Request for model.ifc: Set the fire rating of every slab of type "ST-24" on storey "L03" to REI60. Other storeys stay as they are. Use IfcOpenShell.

First a look at what the model holds.

```python
import ifcopenshell
import ifcopenshell.util.element

model = ifcopenshell.open("model.ifc")
print(model.schema)
storey = next(s for s in model.by_type("IfcBuildingStorey") if s.Name == "L03")
slabs = [e for e in ifcopenshell.util.element.get_decomposition(storey) if e.is_a("IfcSlab")]
seen = {}
for e in slabs:
    element_type = ifcopenshell.util.element.get_type(e)
    key = (element_type.Name if element_type != e and element_type else None, ifcopenshell.util.element.get_pset(e, "Pset_SlabCommon", "FireRating"))
    seen[key] = seen.get(key, 0) + 1
for (name, value), count in sorted(seen.items(), key=str):
    print(count, "x", name, "|", value)
```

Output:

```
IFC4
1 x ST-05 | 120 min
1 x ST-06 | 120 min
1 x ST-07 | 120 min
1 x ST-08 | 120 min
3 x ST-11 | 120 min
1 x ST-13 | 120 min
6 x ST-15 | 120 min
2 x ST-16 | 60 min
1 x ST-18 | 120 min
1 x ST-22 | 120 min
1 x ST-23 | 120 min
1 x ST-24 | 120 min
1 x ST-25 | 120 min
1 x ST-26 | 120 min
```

```python
import ifcopenshell
import ifcopenshell.api.pset
import ifcopenshell.util.element

model = ifcopenshell.open("model.ifc")

storey = next(s for s in model.by_type("IfcBuildingStorey") if s.Name == "L03")
slabs = [e for e in ifcopenshell.util.element.get_decomposition(storey) if e.is_a("IfcSlab")]

count = 0
for e in slabs:
    element_type = ifcopenshell.util.element.get_type(e)
    if element_type in (None, e) or element_type.Name != "ST-24":
        continue
    # add_pset returns the element's existing set when there is one.
    pset = ifcopenshell.api.pset.add_pset(model, product=e, name="Pset_SlabCommon")
    ifcopenshell.api.pset.edit_pset(model, pset=pset, properties={"FireRating": "REI60"})
    count += 1

print(count, "slabs updated")

model.write("model_edited.ifc")
```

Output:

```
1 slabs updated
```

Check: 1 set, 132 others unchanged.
